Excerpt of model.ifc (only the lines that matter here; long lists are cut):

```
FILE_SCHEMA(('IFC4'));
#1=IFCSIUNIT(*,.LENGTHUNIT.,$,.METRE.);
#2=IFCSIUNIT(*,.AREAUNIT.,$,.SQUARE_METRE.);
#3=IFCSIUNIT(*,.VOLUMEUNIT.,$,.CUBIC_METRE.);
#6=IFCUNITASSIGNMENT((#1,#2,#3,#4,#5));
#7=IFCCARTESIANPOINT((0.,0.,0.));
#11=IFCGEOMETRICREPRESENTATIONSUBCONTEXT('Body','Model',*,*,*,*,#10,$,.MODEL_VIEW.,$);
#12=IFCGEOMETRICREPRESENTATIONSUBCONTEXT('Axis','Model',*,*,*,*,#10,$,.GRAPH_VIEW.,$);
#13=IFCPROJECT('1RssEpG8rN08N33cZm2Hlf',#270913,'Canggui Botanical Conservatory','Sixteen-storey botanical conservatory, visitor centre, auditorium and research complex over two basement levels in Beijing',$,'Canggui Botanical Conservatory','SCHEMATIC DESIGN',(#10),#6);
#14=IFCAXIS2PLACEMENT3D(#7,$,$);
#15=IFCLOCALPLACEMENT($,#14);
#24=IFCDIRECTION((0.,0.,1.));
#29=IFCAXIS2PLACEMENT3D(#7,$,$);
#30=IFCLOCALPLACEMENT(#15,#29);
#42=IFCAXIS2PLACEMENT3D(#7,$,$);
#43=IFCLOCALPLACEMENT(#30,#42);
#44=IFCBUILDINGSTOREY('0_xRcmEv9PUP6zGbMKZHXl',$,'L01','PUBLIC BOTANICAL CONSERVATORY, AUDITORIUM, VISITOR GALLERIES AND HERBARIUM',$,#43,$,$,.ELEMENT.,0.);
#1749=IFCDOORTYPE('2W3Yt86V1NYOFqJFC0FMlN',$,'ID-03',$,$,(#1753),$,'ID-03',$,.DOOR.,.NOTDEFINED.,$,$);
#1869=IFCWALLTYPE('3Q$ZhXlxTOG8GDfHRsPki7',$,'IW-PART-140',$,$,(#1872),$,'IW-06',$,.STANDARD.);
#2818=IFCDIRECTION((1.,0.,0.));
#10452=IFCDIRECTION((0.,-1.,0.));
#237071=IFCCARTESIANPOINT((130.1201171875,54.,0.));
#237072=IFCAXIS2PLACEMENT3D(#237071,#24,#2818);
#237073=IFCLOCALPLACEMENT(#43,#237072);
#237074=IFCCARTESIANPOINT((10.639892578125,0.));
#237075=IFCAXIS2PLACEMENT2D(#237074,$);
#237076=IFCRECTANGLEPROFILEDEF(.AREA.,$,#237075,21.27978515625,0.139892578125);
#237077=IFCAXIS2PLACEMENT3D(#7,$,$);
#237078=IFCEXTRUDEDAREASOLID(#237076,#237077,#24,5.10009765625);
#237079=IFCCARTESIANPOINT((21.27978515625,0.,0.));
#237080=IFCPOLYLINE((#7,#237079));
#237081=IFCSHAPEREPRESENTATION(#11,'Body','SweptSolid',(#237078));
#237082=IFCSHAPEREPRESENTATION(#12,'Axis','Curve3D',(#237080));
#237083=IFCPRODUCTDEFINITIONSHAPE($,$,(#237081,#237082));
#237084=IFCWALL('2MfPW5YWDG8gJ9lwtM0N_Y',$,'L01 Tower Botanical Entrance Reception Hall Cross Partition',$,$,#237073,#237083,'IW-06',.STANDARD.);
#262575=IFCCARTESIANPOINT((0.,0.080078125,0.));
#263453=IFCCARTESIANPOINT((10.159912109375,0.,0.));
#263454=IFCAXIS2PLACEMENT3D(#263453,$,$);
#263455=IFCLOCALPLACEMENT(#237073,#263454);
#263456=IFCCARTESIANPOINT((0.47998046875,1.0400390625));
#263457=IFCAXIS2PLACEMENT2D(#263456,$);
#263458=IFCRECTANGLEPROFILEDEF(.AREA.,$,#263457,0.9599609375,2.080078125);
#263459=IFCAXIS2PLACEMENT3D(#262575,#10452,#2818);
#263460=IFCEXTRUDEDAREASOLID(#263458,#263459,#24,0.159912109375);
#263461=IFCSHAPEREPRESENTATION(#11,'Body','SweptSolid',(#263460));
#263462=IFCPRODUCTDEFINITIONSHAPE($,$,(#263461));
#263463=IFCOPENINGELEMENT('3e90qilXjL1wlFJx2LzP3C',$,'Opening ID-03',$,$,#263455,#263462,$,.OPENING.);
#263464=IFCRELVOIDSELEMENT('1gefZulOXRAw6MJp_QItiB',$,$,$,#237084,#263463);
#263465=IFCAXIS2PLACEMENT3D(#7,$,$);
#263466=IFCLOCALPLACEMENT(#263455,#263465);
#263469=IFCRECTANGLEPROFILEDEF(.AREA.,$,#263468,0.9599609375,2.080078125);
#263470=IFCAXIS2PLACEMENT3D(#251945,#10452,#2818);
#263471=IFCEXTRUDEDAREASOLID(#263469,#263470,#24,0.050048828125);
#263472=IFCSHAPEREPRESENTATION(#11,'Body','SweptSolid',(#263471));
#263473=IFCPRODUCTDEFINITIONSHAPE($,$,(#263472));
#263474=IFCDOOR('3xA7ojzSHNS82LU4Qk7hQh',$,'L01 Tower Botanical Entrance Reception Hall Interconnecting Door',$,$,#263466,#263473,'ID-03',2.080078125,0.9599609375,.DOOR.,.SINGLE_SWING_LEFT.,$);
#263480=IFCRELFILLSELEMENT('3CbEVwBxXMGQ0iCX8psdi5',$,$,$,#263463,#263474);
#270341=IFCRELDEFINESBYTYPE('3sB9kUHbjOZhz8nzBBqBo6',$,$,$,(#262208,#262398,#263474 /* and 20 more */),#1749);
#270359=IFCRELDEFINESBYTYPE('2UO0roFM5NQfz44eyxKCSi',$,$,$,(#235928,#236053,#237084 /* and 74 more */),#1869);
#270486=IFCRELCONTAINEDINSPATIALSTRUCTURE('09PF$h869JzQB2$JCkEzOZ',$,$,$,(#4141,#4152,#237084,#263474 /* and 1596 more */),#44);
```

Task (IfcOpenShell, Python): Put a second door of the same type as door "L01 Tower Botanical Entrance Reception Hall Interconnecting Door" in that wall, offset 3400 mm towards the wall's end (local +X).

```python
import ifcopenshell
import ifcopenshell.api.feature
import ifcopenshell.api.geometry
import ifcopenshell.api.root
import ifcopenshell.geom
import ifcopenshell.util.element
import ifcopenshell.util.placement
import ifcopenshell.util.shape
import ifcopenshell.util.unit

model = ifcopenshell.open("model.ifc")
unit_scale = ifcopenshell.util.unit.calculate_unit_scale(model)
settings = ifcopenshell.geom.settings()


def volume(element):
    """Net volume in cubic metres, openings subtracted."""
    shape = ifcopenshell.geom.create_shape(settings, element)
    return ifcopenshell.util.shape.get_volume(shape.geometry)


door = model.by_guid("3xA7ojzSHNS82LU4Qk7hQh")
opening = door.FillsVoids[0].RelatingOpeningElement
wall = opening.VoidsElements[0].RelatingBuildingElement
before = volume(wall)
shift = ifcopenshell.util.placement.get_local_placement(wall.ObjectPlacement)[:3, 0] * 3.4 / unit_scale

# copy_class copies the void relationship, type, container and properties, but no geometry.
new_opening = ifcopenshell.api.root.copy_class(model, product=opening)
new_opening.Representation = ifcopenshell.util.element.copy_deep(
    model, opening.Representation, exclude=["IfcGeometricRepresentationContext", "IfcRepresentationMap"]
)
new_door = ifcopenshell.api.root.copy_class(model, product=door)
new_door.Representation = ifcopenshell.util.element.copy_deep(
    model, door.Representation, exclude=["IfcGeometricRepresentationContext", "IfcRepresentationMap"]
)
new_door.Tag = None
ifcopenshell.api.feature.add_filling(model, opening=new_opening, element=new_door)

for old, new in ((opening, new_opening), (door, new_door)):
    matrix = ifcopenshell.util.placement.get_local_placement(old.ObjectPlacement)
    matrix[:3, 3] += shift
    ifcopenshell.api.geometry.edit_object_placement(model, product=new, matrix=matrix, is_si=False)

after = volume(wall)

print(f"wall volume {before:.3f} -> {after:.3f} m3")

model.write("model_rev.ifc")
```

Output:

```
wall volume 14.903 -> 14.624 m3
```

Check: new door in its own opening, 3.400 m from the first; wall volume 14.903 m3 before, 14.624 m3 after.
